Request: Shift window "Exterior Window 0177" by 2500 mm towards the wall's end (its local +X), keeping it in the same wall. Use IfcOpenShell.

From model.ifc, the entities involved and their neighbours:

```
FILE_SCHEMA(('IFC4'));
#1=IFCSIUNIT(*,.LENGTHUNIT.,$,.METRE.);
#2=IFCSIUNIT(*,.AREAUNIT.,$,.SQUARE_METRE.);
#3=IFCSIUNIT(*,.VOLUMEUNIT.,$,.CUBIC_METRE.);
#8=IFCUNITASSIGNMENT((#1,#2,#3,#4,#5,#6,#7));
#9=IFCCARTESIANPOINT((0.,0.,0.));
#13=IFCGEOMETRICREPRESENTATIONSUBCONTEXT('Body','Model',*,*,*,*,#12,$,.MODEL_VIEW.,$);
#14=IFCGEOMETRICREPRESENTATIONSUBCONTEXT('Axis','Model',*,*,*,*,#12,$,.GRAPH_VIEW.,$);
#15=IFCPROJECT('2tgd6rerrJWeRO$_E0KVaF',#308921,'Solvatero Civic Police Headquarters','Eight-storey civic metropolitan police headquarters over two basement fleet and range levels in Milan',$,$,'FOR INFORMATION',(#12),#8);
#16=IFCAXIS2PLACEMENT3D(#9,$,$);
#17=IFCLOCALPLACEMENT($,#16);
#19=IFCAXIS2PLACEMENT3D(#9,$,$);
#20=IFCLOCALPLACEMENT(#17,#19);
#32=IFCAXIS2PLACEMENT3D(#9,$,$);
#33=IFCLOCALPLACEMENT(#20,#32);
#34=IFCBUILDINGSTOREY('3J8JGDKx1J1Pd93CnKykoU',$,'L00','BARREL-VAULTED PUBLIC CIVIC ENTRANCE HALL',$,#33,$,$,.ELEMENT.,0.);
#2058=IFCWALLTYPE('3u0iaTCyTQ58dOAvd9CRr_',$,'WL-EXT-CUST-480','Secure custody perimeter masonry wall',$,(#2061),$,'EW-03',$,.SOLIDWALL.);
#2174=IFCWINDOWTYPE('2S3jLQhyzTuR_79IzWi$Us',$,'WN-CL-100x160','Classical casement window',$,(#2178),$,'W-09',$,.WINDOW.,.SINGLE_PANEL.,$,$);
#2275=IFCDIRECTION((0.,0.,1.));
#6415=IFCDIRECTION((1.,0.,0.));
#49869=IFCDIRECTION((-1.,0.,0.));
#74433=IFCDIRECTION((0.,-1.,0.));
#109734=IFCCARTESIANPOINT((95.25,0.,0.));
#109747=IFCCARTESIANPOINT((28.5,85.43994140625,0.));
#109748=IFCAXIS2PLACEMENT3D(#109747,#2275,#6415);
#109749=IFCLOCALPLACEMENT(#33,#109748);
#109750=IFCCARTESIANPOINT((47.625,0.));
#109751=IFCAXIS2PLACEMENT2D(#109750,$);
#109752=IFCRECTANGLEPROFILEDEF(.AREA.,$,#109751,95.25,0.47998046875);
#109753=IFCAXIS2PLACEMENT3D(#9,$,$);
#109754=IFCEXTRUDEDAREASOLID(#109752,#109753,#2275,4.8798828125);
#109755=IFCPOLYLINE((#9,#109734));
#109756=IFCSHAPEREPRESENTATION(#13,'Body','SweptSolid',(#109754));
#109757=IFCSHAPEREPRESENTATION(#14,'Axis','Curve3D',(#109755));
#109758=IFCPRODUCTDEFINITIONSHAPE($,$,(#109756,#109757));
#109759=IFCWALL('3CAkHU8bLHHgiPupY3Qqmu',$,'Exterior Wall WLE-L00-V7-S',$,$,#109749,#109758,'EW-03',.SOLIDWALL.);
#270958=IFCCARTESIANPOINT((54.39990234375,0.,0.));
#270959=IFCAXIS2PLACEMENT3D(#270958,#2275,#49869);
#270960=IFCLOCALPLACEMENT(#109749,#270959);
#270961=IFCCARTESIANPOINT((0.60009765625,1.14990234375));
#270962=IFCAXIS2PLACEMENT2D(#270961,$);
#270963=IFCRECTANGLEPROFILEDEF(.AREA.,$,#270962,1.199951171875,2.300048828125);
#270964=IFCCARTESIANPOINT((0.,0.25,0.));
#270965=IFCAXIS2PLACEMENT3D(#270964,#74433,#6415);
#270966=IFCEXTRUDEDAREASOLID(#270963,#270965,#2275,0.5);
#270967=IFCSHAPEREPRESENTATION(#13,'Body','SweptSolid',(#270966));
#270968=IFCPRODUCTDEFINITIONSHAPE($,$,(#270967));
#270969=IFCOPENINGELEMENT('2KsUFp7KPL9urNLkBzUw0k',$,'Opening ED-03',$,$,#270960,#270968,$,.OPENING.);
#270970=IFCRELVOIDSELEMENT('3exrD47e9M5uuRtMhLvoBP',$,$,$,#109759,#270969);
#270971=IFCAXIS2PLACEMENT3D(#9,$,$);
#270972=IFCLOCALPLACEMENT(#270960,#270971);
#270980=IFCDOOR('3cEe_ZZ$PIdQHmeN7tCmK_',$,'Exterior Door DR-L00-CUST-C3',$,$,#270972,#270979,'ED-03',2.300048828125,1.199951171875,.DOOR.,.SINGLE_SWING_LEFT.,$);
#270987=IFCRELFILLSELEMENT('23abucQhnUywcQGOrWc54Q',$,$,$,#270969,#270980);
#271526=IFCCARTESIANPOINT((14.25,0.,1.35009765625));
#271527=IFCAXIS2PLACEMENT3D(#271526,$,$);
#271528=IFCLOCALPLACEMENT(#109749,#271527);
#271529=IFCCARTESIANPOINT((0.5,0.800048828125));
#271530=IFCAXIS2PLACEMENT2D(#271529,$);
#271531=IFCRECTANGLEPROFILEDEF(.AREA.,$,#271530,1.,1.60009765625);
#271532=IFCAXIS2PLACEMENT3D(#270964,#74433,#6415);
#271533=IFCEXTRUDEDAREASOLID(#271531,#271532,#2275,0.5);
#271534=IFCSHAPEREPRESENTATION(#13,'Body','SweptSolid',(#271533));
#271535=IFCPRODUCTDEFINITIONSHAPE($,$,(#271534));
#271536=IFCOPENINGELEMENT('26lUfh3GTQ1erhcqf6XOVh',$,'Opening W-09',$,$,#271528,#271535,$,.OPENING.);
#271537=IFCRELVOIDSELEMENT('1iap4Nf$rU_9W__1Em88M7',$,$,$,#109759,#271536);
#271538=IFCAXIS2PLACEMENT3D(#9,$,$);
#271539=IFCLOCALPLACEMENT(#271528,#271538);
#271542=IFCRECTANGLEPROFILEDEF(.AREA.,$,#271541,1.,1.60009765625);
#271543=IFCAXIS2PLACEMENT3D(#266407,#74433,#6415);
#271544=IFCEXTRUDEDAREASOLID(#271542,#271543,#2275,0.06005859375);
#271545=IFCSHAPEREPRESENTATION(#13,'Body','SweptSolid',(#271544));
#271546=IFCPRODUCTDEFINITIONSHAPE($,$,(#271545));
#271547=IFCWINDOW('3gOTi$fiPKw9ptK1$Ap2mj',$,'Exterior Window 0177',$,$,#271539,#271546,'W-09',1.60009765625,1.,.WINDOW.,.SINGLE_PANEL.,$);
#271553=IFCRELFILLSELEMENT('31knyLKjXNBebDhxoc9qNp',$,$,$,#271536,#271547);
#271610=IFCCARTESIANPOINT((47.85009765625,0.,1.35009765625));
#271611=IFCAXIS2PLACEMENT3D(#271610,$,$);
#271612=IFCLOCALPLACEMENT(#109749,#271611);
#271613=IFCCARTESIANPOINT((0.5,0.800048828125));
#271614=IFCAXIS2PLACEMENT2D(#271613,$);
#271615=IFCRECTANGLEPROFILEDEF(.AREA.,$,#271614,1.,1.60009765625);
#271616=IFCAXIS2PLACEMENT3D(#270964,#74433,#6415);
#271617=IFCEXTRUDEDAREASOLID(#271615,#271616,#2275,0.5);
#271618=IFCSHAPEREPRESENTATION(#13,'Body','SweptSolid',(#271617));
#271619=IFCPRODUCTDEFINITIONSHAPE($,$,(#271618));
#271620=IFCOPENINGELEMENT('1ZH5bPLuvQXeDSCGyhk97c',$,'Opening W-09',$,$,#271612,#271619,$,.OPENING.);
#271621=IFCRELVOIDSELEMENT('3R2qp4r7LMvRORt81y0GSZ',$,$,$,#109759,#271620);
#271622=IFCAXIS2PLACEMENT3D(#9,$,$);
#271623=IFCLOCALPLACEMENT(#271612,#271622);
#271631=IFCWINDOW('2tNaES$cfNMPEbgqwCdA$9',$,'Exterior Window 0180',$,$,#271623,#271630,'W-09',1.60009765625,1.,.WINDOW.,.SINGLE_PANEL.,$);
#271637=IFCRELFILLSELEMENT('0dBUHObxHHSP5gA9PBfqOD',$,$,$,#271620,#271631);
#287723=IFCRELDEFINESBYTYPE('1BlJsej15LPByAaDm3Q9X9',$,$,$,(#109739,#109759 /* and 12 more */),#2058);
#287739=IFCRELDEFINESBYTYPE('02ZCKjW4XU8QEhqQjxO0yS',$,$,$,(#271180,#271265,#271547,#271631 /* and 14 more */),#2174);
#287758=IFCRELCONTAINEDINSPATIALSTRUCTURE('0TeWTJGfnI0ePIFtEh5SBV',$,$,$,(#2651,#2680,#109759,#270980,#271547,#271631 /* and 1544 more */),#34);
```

```python
import ifcopenshell
import ifcopenshell.api.geometry
import ifcopenshell.util.placement

model = ifcopenshell.open("model.ifc")

window = model.by_guid("3gOTi$fiPKw9ptK1$Ap2mj")
opening = window.FillsVoids[0].RelatingOpeningElement
wall = opening.VoidsElements[0].RelatingBuildingElement

wall_matrix = ifcopenshell.util.placement.get_local_placement(wall.ObjectPlacement)
shift = wall_matrix[:3, 0] * 2.5
before = ifcopenshell.util.placement.get_local_placement(window.ObjectPlacement)[:3, 3].copy()

# The window is placed relative to its opening, so it follows when the opening moves.
matrix = ifcopenshell.util.placement.get_local_placement(opening.ObjectPlacement)
matrix[:3, 3] += shift
ifcopenshell.api.geometry.edit_object_placement(
    model, product=opening, matrix=matrix, is_si=False, should_transform_children=True
)

after = ifcopenshell.util.placement.get_local_placement(window.ObjectPlacement)[:3, 3]
print("window moved by", (after - before).round(3) + 0.0)

model.write("model_rev.ifc")
```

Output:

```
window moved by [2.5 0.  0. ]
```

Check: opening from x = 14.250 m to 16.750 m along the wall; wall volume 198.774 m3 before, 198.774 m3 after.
